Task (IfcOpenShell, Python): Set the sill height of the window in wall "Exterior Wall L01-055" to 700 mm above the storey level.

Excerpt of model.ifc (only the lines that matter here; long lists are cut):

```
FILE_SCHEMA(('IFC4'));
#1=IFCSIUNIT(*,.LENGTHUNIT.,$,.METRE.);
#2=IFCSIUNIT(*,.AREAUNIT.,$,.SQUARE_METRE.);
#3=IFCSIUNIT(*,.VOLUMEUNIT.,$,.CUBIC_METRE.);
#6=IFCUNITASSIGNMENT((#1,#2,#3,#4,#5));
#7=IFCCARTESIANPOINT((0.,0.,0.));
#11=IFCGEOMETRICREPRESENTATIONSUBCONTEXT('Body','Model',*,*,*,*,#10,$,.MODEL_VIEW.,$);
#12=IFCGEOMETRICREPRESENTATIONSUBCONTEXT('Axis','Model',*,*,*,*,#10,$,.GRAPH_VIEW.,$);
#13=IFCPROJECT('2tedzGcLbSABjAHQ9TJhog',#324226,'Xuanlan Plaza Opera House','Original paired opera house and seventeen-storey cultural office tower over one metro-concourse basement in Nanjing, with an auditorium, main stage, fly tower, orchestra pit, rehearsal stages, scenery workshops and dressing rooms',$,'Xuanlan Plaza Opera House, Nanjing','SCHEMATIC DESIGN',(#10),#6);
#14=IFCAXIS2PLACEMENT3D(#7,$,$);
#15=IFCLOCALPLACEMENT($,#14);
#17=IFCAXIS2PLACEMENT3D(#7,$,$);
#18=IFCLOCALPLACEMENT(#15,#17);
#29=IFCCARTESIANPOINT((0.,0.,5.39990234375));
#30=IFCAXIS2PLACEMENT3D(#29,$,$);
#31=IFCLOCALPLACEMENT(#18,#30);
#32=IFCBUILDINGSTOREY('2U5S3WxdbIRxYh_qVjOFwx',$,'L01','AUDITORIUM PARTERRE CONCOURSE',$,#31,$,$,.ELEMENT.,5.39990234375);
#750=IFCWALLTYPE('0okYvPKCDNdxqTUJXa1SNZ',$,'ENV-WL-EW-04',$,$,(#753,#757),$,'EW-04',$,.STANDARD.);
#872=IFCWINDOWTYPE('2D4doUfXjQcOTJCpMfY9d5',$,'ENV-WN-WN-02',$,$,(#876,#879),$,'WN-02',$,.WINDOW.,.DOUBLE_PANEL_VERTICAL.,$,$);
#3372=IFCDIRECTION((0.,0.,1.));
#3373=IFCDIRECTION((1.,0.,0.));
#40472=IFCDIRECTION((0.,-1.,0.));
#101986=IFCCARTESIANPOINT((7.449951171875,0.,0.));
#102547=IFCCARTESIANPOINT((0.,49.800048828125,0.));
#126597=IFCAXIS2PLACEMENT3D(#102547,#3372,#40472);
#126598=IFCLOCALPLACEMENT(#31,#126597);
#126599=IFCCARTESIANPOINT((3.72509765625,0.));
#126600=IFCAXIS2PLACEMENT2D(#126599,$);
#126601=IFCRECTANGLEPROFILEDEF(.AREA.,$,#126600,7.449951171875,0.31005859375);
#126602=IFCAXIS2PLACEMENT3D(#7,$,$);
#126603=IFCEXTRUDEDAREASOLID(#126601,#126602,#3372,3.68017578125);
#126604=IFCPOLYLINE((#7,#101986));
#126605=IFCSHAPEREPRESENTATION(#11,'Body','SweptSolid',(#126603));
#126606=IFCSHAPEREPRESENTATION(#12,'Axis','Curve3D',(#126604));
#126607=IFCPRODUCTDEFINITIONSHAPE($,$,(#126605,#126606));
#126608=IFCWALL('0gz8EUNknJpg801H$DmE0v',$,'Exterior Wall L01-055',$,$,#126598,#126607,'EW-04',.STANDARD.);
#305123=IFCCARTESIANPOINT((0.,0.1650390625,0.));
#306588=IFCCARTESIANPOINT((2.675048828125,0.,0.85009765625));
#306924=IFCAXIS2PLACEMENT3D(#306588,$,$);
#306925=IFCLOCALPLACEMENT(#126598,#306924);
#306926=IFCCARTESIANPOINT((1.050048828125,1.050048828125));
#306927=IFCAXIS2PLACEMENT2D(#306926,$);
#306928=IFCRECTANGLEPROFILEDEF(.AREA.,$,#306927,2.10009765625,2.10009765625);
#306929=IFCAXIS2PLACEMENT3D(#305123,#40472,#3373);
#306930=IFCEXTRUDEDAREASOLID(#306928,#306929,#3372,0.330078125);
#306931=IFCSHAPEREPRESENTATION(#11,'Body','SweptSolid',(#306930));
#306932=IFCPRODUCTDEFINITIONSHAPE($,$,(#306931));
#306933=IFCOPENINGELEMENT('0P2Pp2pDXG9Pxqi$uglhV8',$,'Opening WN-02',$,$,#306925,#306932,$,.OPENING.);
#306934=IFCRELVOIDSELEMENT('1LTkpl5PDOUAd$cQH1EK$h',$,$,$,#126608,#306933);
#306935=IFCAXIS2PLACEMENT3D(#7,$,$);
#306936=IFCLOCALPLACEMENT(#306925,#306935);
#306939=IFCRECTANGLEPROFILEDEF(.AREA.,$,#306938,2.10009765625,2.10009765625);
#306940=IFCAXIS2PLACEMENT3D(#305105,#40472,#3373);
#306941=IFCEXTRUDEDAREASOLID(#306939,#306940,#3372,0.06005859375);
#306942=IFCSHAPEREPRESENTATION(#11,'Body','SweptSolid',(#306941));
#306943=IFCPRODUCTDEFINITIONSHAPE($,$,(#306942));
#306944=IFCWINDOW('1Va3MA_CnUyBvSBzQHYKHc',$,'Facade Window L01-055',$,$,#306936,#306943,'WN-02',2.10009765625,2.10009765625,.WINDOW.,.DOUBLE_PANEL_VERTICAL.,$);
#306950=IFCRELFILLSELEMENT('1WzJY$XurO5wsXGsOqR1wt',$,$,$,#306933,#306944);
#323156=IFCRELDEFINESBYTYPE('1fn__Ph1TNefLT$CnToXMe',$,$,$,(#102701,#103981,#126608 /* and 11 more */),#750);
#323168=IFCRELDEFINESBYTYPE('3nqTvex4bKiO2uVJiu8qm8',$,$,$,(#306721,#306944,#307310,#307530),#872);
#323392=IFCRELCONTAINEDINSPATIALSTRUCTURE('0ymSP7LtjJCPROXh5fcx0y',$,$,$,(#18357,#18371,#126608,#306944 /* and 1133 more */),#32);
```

```python
import numpy as np
import ifcopenshell
import ifcopenshell.api.geometry
import ifcopenshell.geom
import ifcopenshell.util.element
import ifcopenshell.util.placement
import ifcopenshell.util.shape
import ifcopenshell.util.unit

model = ifcopenshell.open("model.ifc")
unit_scale = ifcopenshell.util.unit.calculate_unit_scale(model)

window = model.by_id(306944)
opening = window.FillsVoids[0].RelatingOpeningElement
storey = ifcopenshell.util.element.get_container(window, ifc_class="IfcBuildingStorey")
level = ifcopenshell.util.placement.get_local_placement(storey.ObjectPlacement)[2, 3]

# The opening's origin need not be at the sill, so measure its lowest point.
shape = ifcopenshell.geom.create_shape(ifcopenshell.geom.settings(), opening)
bottom = ifcopenshell.util.shape.get_shape_bottom_elevation(shape, shape.geometry) / unit_scale
dz = level + 0.7 / unit_scale - bottom

shift = np.array([0.0, 0.0, dz])
# The window is placed relative to its opening, so it follows when the opening moves.
matrix = ifcopenshell.util.placement.get_local_placement(opening.ObjectPlacement)
matrix[:3, 3] += shift
ifcopenshell.api.geometry.edit_object_placement(
    model, product=opening, matrix=matrix, is_si=False, should_transform_children=True
)

print(f"moved by {dz * unit_scale:+.3f} m")

model.write("model_rev.ifc")
```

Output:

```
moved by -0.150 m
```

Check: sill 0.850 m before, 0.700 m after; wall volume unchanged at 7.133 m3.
